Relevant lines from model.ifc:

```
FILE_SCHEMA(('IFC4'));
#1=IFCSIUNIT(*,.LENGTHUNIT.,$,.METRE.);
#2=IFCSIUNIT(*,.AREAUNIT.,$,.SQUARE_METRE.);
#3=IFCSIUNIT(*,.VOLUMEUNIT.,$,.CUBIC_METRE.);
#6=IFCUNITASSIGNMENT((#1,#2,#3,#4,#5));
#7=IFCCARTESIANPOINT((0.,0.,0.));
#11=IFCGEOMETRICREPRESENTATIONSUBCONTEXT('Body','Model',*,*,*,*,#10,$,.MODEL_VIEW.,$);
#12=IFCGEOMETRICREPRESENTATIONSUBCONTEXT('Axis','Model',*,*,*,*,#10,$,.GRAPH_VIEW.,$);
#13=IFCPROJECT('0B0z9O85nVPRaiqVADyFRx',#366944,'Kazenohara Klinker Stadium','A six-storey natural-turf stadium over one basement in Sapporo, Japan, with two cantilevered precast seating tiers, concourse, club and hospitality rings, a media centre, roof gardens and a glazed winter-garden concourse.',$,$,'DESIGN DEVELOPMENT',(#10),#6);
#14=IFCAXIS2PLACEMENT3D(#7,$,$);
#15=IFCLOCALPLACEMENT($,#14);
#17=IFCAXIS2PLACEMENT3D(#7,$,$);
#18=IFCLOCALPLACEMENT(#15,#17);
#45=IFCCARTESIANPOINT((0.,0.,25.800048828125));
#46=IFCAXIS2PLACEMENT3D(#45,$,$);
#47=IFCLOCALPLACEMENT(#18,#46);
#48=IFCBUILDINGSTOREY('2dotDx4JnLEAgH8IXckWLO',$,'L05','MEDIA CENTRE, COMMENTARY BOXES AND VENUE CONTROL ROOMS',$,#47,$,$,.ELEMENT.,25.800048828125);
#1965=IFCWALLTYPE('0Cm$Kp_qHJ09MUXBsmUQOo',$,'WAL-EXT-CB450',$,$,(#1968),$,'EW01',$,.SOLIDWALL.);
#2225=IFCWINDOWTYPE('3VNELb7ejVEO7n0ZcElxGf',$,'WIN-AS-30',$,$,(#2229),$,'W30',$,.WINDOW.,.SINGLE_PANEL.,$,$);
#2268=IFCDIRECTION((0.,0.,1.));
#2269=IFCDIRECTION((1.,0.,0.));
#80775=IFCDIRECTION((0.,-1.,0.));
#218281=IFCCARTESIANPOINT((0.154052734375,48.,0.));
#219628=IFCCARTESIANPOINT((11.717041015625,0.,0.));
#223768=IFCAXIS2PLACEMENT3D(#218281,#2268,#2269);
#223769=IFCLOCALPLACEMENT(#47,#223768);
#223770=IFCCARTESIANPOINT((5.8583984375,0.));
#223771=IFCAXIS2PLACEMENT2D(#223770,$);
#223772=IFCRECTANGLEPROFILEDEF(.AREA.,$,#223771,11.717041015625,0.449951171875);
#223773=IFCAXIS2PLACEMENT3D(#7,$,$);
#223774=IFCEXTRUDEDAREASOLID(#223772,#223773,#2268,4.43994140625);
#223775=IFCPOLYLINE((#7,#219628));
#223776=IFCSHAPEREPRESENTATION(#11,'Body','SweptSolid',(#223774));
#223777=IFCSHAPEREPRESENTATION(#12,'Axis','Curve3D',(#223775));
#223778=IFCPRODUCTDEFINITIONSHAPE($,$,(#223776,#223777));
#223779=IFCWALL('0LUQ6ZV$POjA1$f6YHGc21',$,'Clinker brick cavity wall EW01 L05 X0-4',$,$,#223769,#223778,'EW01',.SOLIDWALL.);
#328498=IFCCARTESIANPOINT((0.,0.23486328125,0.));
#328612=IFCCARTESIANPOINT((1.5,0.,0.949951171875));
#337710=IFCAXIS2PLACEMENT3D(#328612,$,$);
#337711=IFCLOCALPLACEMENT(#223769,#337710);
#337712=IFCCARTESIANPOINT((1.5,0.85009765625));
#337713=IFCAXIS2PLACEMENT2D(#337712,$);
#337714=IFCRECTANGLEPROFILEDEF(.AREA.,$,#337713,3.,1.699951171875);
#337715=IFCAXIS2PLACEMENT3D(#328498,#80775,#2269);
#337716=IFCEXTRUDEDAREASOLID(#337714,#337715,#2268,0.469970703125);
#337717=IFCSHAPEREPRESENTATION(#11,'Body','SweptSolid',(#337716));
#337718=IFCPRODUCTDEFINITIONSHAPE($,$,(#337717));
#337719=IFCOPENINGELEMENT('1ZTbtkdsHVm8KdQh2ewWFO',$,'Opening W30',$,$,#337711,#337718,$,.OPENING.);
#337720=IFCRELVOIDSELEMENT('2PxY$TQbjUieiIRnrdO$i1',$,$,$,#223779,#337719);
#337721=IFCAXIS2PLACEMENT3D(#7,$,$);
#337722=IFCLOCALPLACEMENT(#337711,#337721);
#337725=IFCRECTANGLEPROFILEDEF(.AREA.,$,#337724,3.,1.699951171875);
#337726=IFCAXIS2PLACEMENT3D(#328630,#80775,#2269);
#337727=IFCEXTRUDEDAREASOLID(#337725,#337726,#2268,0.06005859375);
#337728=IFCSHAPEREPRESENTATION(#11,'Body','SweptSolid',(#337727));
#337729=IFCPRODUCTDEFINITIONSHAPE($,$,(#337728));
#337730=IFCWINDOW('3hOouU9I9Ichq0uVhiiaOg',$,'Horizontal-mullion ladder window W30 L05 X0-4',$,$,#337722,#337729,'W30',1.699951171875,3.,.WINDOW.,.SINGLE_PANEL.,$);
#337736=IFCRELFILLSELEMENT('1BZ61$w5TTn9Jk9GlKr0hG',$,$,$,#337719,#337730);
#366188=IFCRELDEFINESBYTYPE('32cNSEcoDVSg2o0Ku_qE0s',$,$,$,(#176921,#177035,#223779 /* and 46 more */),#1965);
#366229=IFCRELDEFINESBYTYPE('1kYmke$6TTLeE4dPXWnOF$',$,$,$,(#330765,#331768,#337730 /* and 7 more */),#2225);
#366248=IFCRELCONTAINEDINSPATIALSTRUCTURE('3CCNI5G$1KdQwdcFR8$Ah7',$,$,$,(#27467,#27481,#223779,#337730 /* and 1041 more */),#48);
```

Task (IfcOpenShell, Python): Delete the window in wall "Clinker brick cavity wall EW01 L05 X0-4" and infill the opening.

```python
import ifcopenshell
import ifcopenshell.api.feature
import ifcopenshell.api.root
import ifcopenshell.geom
import ifcopenshell.util.shape

model = ifcopenshell.open("model.ifc")
settings = ifcopenshell.geom.settings()


def volume(element):
    """Net volume in cubic metres, openings subtracted."""
    shape = ifcopenshell.geom.create_shape(settings, element)
    return ifcopenshell.util.shape.get_volume(shape.geometry)


window = model.by_guid("3hOouU9I9Ichq0uVhiiaOg")
opening = window.FillsVoids[0].RelatingOpeningElement
wall = opening.VoidsElements[0].RelatingBuildingElement
before = volume(wall)

ifcopenshell.api.root.remove_product(model, product=window)
ifcopenshell.api.feature.remove_feature(model, feature=opening)

after = volume(wall)

print(f"wall volume {before:.3f} -> {after:.3f} m3")

model.write("model_updated.ifc")
```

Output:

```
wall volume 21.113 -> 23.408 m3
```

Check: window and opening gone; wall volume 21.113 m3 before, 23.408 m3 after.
